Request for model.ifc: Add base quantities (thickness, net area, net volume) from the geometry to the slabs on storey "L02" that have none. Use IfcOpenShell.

First a look at what the model holds.

```python
import ifcopenshell
import ifcopenshell.util.element
import ifcopenshell.util.unit

model = ifcopenshell.open("model.ifc")
print(model.schema)
for unit_type in ("LENGTHUNIT", "AREAUNIT", "VOLUMEUNIT"):
    print(unit_type, ifcopenshell.util.unit.calculate_unit_scale(model, unit_type))
storey = next(s for s in model.by_type("IfcBuildingStorey") if s.Name == "L02")
slabs = [e for e in ifcopenshell.util.element.get_decomposition(storey) if e.is_a("IfcSlab")]
for e in sorted(slabs, key=lambda e: e.id()):
    print(e.id(), e.is_a(), e.Name, list(ifcopenshell.util.element.get_psets(e, qtos_only=True)), sep=" | ")
```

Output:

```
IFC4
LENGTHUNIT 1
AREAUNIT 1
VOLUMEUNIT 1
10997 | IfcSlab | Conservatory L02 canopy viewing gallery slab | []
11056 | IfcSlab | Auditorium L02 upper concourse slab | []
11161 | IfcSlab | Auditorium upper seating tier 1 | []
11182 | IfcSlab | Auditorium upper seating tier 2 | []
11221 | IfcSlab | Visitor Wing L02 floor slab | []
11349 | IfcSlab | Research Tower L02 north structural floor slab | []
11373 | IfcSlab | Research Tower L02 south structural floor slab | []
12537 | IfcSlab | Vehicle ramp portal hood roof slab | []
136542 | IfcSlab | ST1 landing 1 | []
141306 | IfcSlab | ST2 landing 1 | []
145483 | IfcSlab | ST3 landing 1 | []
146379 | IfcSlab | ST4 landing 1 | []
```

```python
import ifcopenshell
import ifcopenshell.api.pset
import ifcopenshell.geom
import ifcopenshell.util.element
import ifcopenshell.util.shape
import ifcopenshell.util.unit

model = ifcopenshell.open("model.ifc")
unit_scale = ifcopenshell.util.unit.calculate_unit_scale(model)
area_scale = ifcopenshell.util.unit.calculate_unit_scale(model, "AREAUNIT")
volume_scale = ifcopenshell.util.unit.calculate_unit_scale(model, "VOLUMEUNIT")
settings = ifcopenshell.geom.settings()

storey = next(s for s in model.by_type("IfcBuildingStorey") if s.Name == "L02")
slabs = [e for e in ifcopenshell.util.element.get_decomposition(storey) if e.is_a("IfcSlab")]

for e in sorted(slabs, key=lambda e: e.id()):
    if ifcopenshell.util.element.get_psets(e, qtos_only=True, should_inherit=False):
        continue
    # Geometry comes back in metres, in the element's own axes.
    shape = ifcopenshell.geom.create_shape(settings, e)
    values = {
        "Width": ifcopenshell.util.shape.get_z(shape.geometry) / unit_scale,
        "NetArea": ifcopenshell.util.shape.get_footprint_area(shape.geometry) / area_scale,
        "NetVolume": ifcopenshell.util.shape.get_volume(shape.geometry) / volume_scale,
    }
    qto = ifcopenshell.api.pset.add_qto(model, product=e, name="Qto_SlabBaseQuantities")
    ifcopenshell.api.pset.edit_qto(model, qto=qto, properties=values)
    print(e.id(), {k: round(v, 3) for k, v in values.items()})

model.write("model_rev.ifc")
```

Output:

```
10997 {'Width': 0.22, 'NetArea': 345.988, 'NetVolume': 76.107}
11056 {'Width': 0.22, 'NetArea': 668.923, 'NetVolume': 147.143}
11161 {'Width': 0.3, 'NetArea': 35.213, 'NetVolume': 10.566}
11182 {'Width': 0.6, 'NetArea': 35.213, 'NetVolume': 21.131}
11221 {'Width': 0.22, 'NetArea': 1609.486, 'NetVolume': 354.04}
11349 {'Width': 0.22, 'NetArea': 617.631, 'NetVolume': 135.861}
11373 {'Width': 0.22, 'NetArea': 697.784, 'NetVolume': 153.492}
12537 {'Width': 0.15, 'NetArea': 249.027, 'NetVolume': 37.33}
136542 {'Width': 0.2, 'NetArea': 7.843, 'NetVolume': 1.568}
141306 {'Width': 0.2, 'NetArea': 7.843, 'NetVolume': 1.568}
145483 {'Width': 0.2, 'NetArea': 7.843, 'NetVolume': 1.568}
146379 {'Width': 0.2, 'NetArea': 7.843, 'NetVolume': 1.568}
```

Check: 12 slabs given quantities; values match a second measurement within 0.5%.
